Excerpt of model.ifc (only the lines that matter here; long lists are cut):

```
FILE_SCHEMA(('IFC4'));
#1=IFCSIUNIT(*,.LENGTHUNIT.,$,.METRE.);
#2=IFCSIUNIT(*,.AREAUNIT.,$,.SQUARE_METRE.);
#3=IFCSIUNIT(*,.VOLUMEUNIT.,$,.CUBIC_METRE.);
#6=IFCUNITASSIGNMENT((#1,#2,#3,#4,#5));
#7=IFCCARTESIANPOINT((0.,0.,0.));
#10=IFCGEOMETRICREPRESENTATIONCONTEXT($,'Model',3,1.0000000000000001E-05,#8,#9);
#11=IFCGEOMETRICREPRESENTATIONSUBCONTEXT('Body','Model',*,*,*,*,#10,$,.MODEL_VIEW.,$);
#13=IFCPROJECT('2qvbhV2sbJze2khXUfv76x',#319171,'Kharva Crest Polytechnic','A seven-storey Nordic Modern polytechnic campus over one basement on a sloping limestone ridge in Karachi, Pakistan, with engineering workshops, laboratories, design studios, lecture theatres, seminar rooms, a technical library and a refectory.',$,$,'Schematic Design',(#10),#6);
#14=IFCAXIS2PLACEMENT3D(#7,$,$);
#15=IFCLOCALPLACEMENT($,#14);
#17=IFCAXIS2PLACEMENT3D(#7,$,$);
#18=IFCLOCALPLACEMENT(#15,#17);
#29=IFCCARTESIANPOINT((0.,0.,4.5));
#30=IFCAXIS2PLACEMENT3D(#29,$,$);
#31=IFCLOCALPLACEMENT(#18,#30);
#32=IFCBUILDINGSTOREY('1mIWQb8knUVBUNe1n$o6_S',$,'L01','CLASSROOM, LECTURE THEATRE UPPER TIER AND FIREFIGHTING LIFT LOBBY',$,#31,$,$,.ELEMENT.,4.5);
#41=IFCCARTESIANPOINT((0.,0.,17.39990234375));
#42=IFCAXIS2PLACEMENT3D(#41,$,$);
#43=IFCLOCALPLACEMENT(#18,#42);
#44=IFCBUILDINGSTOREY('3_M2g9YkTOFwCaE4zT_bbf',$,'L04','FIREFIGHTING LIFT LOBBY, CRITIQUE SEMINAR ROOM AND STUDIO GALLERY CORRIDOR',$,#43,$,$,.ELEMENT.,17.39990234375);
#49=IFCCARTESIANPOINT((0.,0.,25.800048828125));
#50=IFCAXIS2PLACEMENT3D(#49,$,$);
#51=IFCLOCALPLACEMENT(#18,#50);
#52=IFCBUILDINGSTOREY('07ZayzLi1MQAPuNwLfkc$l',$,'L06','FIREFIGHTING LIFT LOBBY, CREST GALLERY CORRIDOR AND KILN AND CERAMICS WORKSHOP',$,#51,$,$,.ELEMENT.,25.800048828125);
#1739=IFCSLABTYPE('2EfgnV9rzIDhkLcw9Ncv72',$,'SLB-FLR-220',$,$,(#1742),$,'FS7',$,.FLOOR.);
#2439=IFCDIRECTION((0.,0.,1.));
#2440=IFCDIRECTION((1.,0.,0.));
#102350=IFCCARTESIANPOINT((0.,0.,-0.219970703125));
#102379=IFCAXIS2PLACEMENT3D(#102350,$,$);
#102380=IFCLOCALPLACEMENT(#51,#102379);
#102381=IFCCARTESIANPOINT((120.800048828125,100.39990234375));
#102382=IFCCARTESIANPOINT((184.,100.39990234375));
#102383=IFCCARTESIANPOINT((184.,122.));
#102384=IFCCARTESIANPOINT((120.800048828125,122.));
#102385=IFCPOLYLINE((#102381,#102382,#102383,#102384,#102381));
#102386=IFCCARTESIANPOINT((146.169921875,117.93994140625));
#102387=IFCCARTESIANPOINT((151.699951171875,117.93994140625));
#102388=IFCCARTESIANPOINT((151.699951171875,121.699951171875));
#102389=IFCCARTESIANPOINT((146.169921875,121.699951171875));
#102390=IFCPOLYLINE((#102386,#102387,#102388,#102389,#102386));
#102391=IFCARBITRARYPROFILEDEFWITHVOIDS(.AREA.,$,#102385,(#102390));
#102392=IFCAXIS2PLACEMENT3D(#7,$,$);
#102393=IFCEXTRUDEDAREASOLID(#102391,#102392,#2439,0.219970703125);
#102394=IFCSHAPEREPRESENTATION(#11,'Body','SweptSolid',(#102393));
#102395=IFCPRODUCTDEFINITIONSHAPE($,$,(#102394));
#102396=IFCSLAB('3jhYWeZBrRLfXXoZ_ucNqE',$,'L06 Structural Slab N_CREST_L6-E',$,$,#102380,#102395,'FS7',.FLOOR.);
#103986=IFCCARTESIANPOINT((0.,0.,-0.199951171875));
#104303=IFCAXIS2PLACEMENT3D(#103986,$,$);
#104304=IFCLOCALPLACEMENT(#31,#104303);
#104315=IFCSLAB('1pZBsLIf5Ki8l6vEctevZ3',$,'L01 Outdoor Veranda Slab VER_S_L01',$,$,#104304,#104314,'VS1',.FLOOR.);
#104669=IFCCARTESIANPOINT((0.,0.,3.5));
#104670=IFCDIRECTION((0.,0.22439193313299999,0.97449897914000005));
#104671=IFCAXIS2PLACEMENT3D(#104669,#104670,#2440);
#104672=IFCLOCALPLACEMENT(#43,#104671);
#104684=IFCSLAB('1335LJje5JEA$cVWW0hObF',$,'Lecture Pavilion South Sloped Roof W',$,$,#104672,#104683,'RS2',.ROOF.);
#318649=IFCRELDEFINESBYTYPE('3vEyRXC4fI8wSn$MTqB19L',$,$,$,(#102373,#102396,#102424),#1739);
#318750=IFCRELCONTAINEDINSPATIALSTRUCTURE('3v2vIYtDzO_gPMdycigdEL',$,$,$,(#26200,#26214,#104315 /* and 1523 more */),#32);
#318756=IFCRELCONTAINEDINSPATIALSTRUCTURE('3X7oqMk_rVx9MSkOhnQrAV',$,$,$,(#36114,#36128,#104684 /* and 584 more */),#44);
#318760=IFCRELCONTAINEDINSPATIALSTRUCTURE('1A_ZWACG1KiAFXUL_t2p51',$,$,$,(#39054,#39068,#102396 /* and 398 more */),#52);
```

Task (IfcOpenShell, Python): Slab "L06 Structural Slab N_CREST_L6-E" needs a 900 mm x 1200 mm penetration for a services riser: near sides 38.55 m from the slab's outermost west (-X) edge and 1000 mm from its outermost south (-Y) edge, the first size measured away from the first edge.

```python
import numpy as np
import ifcopenshell
import ifcopenshell.api.feature
import ifcopenshell.api.geometry
import ifcopenshell.api.root
import ifcopenshell.geom
import ifcopenshell.util.placement
import ifcopenshell.util.representation
import ifcopenshell.util.shape
import ifcopenshell.util.unit

model = ifcopenshell.open("model.ifc")
unit_scale = ifcopenshell.util.unit.calculate_unit_scale(model)
settings = ifcopenshell.geom.settings()


def volume(element):
    """Net volume in cubic metres, openings subtracted."""
    shape = ifcopenshell.geom.create_shape(settings, element)
    return ifcopenshell.util.shape.get_volume(shape.geometry)


slab = model.by_id(102396)
before = volume(slab)

# Extent in the slab's own axes, in metres. The edges named are its -X and -Y sides.
slab_shape = ifcopenshell.geom.create_shape(settings, slab)
vertices = ifcopenshell.util.shape.get_vertices(slab_shape.geometry)
x_min, y_min, bottom = vertices.min(axis=0)
top = vertices[:, 2].max()

opening = ifcopenshell.api.root.create_entity(model, ifc_class="IfcOpeningElement", name="Services riser opening", predefined_type="OPENING")
context = ifcopenshell.util.representation.get_context(model, "Model", "Body", "MODEL_VIEW")
width, depth = 0.9, 1.2
outline = [(0.0, 0.0), (width, 0.0), (width, depth), (0.0, depth), (0.0, 0.0)]
# Overshoot both faces by 50 mm so the cut is clean.
shape = ifcopenshell.api.geometry.add_slab_representation(
    model, context=context, depth=top - bottom + 0.1, polyline=outline
)
ifcopenshell.api.geometry.assign_representation(model, product=opening, representation=shape)

matrix = ifcopenshell.util.placement.get_local_placement(slab.ObjectPlacement)
matrix[:, 3] = matrix @ np.append(np.array([x_min + 38.55, y_min + 1, bottom - 0.05]) / unit_scale, 1.0)
ifcopenshell.api.geometry.edit_object_placement(model, product=opening, matrix=matrix, is_si=False)
ifcopenshell.api.feature.add_feature(model, feature=opening, element=slab)

after = volume(slab)

print(f"slab volume {before:.3f} -> {after:.3f} m3")

model.write("model-out.ifc")
```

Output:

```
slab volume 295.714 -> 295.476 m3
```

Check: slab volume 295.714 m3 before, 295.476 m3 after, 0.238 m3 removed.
